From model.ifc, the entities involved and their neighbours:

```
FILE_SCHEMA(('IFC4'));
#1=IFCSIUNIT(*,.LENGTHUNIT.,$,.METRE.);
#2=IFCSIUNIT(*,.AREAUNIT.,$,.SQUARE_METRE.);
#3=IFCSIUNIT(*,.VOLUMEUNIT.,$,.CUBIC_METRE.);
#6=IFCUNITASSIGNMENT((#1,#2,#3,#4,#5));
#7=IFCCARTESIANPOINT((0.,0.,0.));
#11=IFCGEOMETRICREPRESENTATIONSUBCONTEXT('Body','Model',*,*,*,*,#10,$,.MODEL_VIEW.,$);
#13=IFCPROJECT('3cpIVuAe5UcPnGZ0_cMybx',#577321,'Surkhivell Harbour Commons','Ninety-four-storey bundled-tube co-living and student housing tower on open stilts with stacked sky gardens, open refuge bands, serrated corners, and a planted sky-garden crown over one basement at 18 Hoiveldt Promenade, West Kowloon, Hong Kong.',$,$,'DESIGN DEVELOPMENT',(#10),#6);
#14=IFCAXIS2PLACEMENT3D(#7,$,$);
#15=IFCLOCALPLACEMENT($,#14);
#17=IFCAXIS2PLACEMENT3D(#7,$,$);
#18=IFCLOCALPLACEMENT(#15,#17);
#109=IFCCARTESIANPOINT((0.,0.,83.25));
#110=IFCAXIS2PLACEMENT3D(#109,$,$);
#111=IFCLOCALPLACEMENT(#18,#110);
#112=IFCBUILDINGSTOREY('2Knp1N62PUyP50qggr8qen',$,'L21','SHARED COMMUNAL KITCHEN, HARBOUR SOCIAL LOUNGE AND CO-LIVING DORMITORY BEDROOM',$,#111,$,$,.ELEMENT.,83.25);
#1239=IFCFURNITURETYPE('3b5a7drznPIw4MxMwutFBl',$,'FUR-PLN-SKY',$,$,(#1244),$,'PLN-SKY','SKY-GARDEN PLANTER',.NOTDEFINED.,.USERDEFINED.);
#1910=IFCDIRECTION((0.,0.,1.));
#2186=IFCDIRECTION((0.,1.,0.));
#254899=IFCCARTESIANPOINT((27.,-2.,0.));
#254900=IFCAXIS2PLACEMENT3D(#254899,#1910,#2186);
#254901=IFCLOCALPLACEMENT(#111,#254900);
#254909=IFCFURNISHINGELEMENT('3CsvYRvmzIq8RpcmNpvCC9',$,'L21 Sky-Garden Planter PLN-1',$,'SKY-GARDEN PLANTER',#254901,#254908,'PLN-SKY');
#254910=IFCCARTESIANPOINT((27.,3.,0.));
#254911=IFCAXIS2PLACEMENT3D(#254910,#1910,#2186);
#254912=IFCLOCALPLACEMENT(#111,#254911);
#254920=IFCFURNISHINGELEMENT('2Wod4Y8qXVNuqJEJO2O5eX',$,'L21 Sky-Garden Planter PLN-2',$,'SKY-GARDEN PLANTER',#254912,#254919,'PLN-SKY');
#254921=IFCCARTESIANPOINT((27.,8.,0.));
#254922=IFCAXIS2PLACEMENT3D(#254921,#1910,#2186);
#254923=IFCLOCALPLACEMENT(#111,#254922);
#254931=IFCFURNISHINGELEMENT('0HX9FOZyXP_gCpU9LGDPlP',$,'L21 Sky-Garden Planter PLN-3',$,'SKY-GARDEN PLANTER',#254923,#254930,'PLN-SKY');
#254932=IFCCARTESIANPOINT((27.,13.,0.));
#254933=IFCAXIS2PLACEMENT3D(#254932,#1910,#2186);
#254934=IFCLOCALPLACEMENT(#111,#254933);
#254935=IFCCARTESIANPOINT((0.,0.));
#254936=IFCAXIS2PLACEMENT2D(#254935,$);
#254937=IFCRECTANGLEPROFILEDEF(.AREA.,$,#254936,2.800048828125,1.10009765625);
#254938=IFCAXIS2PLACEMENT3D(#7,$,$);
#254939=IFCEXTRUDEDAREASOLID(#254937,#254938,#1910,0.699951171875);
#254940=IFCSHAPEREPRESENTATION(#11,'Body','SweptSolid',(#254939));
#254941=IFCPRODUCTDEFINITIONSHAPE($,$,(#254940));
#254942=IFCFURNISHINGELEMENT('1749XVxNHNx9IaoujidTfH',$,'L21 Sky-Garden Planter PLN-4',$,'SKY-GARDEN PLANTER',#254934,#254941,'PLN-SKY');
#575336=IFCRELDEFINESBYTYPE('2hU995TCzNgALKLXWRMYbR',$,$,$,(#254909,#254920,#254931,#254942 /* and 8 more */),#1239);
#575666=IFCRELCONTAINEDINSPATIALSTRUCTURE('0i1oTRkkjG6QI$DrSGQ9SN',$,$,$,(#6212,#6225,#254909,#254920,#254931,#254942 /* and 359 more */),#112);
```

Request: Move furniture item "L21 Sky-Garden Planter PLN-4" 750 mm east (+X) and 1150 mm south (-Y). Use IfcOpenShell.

```python
import ifcopenshell
import ifcopenshell.api.geometry
import ifcopenshell.util.placement

model = ifcopenshell.open("model.ifc")

item = model.by_guid("1749XVxNHNx9IaoujidTfH")
matrix = ifcopenshell.util.placement.get_local_placement(item.ObjectPlacement)
matrix[0, 3] += 0.75
matrix[1, 3] -= 1.15
ifcopenshell.api.geometry.edit_object_placement(model, product=item, matrix=matrix, is_si=False)

print(ifcopenshell.util.placement.get_local_placement(item.ObjectPlacement).round(3) + 0.0)

model.write("model-out.ifc")
```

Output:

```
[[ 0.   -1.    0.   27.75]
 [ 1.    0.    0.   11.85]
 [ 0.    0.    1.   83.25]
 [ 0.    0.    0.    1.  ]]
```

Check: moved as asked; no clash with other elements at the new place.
